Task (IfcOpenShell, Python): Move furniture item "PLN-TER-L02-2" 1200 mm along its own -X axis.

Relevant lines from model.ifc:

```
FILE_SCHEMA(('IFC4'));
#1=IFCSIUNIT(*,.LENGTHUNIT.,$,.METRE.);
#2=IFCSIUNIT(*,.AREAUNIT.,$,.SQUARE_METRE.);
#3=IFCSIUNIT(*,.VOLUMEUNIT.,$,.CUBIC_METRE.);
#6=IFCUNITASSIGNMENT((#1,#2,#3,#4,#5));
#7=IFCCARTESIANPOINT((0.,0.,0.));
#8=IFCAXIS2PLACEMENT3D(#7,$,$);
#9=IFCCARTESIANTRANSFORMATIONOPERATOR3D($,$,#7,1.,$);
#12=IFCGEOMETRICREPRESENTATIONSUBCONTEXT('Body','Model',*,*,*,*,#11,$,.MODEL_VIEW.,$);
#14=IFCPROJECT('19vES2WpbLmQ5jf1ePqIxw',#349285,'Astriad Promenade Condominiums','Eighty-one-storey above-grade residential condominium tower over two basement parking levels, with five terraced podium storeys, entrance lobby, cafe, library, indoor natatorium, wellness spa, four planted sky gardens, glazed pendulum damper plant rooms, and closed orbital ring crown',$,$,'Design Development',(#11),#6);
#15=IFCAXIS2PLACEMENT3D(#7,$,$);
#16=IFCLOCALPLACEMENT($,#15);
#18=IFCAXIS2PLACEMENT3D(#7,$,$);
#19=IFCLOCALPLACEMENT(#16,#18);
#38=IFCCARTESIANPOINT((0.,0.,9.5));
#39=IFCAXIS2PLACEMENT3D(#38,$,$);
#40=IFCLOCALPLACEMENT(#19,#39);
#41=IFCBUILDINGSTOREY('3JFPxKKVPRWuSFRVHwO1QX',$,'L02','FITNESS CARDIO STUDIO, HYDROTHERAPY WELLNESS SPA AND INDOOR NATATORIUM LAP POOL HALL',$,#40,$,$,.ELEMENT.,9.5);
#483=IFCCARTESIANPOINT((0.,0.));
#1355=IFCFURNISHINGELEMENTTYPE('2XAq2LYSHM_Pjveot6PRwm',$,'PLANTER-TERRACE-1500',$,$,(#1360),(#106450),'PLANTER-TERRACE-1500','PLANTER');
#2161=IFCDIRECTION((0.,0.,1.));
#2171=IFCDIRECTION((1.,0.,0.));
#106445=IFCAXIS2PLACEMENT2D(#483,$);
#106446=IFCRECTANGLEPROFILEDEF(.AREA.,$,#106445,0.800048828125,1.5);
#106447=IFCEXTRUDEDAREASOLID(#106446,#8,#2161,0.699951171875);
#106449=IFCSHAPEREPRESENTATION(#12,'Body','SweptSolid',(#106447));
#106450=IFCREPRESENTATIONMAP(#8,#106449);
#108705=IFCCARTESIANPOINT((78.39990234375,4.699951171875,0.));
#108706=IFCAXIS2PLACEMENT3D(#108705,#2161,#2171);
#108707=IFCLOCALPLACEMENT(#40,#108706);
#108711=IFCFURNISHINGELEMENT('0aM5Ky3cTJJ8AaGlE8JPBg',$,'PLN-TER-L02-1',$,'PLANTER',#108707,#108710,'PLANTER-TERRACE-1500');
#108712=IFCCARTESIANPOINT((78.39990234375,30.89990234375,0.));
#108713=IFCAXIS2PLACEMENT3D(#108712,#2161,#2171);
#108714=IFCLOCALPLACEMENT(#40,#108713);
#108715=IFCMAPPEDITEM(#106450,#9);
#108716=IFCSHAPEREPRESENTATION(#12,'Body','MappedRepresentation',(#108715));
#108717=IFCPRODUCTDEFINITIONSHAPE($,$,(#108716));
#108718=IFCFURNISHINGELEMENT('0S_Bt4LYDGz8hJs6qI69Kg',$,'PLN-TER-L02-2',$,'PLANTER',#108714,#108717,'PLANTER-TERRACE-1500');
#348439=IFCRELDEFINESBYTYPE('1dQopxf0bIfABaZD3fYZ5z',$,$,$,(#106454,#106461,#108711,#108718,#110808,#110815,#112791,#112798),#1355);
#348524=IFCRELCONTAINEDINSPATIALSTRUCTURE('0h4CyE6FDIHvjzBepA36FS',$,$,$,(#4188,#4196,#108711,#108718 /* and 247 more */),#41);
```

```python
import ifcopenshell
import ifcopenshell.api.geometry
import ifcopenshell.util.placement
import ifcopenshell.util.unit

model = ifcopenshell.open("model.ifc")
unit_scale = ifcopenshell.util.unit.calculate_unit_scale(model)

item = model.by_id(108718)
matrix = ifcopenshell.util.placement.get_local_placement(item.ObjectPlacement)
matrix[:3, 3] -= matrix[:3, 0] * 1.2 / unit_scale
ifcopenshell.api.geometry.edit_object_placement(model, product=item, matrix=matrix, is_si=False)

print(ifcopenshell.util.placement.get_local_placement(item.ObjectPlacement).round(3) + 0.0)

model.write("model_updated.ifc")
```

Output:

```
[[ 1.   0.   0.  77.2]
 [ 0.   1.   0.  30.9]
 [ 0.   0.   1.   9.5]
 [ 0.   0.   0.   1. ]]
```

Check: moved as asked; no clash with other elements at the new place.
